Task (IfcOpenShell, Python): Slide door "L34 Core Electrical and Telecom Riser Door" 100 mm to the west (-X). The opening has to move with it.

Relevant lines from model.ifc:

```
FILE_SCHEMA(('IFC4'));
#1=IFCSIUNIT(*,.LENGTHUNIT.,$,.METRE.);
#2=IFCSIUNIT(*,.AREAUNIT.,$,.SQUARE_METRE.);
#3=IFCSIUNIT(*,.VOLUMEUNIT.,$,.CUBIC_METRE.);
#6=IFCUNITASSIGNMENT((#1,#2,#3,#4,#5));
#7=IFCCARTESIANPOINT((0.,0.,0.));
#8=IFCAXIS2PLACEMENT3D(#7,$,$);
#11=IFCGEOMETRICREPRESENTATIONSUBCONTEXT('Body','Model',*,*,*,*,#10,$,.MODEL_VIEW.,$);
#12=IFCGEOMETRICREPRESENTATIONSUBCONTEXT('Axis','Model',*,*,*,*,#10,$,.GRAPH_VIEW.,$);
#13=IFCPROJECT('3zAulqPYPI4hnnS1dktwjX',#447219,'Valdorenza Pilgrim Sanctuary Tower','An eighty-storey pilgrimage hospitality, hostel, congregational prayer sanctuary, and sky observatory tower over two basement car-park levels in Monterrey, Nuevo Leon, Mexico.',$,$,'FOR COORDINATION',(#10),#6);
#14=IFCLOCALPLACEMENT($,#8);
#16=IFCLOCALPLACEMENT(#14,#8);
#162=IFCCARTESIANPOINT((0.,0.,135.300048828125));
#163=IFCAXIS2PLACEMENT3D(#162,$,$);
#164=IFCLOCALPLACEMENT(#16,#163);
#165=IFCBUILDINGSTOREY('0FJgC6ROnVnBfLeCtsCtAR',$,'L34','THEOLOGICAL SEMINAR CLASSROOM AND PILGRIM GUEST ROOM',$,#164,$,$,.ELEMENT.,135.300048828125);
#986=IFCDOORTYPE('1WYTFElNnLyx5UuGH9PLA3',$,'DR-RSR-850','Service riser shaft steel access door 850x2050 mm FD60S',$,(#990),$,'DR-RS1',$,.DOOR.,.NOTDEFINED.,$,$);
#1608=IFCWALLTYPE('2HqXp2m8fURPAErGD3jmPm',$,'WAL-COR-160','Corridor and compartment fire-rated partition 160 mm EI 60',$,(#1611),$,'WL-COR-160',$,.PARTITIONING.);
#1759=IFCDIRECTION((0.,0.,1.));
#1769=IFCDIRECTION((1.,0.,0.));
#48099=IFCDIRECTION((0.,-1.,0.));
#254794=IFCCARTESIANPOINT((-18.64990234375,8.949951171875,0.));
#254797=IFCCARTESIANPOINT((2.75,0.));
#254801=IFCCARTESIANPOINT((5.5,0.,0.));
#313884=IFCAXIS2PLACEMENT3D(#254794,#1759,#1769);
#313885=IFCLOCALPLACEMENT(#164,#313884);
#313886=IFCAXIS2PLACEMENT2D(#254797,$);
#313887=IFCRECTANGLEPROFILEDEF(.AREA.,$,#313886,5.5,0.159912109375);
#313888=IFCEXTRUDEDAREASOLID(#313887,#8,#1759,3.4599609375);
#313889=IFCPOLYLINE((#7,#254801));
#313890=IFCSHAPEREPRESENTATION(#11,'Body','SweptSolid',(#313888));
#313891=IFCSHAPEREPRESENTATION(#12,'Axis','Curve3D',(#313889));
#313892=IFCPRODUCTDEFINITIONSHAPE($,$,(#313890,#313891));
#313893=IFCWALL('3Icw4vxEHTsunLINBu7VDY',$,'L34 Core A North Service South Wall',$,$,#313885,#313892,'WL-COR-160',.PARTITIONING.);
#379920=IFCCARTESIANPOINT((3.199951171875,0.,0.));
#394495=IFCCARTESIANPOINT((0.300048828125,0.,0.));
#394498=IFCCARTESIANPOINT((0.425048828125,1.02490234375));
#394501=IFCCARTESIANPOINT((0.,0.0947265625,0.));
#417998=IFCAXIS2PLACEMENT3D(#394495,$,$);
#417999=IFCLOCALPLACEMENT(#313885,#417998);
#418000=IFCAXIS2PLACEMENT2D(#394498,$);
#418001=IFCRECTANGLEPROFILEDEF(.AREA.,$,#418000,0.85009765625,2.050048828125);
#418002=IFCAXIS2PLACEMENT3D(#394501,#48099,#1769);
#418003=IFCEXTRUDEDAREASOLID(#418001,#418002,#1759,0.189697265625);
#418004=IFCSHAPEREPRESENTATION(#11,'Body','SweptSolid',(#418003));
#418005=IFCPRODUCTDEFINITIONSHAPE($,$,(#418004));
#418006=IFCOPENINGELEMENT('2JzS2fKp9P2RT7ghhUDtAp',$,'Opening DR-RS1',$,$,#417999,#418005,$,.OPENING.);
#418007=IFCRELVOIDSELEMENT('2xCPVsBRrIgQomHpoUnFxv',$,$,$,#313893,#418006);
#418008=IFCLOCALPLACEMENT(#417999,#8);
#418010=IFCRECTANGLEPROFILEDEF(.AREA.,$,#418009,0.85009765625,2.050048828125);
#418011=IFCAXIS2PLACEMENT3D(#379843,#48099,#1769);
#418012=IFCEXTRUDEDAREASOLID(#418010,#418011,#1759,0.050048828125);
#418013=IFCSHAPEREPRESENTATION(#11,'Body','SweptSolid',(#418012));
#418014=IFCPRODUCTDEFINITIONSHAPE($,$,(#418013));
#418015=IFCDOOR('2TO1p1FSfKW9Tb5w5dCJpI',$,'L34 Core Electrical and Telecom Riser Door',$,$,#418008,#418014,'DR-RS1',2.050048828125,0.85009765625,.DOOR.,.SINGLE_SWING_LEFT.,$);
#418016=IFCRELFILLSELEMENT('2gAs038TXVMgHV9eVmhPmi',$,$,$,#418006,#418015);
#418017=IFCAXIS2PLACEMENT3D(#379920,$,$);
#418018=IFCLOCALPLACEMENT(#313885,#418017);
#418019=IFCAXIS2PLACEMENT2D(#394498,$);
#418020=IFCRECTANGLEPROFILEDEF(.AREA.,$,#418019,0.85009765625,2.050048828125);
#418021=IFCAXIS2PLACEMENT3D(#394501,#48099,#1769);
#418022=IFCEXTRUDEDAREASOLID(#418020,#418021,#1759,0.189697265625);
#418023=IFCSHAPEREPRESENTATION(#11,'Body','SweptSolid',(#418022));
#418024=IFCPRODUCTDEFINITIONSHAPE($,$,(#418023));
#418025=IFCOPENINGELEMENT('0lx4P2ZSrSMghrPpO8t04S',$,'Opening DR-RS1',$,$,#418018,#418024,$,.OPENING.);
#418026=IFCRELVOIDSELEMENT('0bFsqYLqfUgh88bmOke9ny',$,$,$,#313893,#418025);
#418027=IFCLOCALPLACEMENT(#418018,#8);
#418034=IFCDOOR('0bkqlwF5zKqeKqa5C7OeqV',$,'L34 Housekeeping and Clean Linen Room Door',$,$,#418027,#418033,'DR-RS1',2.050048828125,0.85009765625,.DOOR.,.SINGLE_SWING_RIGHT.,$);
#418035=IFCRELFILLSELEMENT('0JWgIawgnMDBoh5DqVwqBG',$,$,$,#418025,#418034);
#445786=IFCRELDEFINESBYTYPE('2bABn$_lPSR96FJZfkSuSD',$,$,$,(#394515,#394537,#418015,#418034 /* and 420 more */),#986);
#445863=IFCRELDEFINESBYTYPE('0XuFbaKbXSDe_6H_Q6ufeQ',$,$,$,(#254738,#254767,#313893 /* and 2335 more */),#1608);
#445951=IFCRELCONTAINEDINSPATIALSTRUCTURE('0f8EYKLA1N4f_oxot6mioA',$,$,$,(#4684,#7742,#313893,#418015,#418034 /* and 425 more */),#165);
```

```python
import ifcopenshell
import ifcopenshell.api.geometry
import ifcopenshell.util.placement
import ifcopenshell.util.unit

model = ifcopenshell.open("model.ifc")
unit_scale = ifcopenshell.util.unit.calculate_unit_scale(model)

door = model.by_guid("2TO1p1FSfKW9Tb5w5dCJpI")
opening = door.FillsVoids[0].RelatingOpeningElement
wall = opening.VoidsElements[0].RelatingBuildingElement

wall_matrix = ifcopenshell.util.placement.get_local_placement(wall.ObjectPlacement)
shift = wall_matrix[:3, 0] * -0.1 / unit_scale
before = ifcopenshell.util.placement.get_local_placement(door.ObjectPlacement)[:3, 3].copy()

# The door is placed relative to its opening, so it follows when the opening moves.
matrix = ifcopenshell.util.placement.get_local_placement(opening.ObjectPlacement)
matrix[:3, 3] += shift
ifcopenshell.api.geometry.edit_object_placement(
    model, product=opening, matrix=matrix, is_si=False, should_transform_children=True
)

after = ifcopenshell.util.placement.get_local_placement(door.ObjectPlacement)[:3, 3]
print("door moved by", (after - before).round(3) + 0.0)

model.write("model_rev.ifc")
```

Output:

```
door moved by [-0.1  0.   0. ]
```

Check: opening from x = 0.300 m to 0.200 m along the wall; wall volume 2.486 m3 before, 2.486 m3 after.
